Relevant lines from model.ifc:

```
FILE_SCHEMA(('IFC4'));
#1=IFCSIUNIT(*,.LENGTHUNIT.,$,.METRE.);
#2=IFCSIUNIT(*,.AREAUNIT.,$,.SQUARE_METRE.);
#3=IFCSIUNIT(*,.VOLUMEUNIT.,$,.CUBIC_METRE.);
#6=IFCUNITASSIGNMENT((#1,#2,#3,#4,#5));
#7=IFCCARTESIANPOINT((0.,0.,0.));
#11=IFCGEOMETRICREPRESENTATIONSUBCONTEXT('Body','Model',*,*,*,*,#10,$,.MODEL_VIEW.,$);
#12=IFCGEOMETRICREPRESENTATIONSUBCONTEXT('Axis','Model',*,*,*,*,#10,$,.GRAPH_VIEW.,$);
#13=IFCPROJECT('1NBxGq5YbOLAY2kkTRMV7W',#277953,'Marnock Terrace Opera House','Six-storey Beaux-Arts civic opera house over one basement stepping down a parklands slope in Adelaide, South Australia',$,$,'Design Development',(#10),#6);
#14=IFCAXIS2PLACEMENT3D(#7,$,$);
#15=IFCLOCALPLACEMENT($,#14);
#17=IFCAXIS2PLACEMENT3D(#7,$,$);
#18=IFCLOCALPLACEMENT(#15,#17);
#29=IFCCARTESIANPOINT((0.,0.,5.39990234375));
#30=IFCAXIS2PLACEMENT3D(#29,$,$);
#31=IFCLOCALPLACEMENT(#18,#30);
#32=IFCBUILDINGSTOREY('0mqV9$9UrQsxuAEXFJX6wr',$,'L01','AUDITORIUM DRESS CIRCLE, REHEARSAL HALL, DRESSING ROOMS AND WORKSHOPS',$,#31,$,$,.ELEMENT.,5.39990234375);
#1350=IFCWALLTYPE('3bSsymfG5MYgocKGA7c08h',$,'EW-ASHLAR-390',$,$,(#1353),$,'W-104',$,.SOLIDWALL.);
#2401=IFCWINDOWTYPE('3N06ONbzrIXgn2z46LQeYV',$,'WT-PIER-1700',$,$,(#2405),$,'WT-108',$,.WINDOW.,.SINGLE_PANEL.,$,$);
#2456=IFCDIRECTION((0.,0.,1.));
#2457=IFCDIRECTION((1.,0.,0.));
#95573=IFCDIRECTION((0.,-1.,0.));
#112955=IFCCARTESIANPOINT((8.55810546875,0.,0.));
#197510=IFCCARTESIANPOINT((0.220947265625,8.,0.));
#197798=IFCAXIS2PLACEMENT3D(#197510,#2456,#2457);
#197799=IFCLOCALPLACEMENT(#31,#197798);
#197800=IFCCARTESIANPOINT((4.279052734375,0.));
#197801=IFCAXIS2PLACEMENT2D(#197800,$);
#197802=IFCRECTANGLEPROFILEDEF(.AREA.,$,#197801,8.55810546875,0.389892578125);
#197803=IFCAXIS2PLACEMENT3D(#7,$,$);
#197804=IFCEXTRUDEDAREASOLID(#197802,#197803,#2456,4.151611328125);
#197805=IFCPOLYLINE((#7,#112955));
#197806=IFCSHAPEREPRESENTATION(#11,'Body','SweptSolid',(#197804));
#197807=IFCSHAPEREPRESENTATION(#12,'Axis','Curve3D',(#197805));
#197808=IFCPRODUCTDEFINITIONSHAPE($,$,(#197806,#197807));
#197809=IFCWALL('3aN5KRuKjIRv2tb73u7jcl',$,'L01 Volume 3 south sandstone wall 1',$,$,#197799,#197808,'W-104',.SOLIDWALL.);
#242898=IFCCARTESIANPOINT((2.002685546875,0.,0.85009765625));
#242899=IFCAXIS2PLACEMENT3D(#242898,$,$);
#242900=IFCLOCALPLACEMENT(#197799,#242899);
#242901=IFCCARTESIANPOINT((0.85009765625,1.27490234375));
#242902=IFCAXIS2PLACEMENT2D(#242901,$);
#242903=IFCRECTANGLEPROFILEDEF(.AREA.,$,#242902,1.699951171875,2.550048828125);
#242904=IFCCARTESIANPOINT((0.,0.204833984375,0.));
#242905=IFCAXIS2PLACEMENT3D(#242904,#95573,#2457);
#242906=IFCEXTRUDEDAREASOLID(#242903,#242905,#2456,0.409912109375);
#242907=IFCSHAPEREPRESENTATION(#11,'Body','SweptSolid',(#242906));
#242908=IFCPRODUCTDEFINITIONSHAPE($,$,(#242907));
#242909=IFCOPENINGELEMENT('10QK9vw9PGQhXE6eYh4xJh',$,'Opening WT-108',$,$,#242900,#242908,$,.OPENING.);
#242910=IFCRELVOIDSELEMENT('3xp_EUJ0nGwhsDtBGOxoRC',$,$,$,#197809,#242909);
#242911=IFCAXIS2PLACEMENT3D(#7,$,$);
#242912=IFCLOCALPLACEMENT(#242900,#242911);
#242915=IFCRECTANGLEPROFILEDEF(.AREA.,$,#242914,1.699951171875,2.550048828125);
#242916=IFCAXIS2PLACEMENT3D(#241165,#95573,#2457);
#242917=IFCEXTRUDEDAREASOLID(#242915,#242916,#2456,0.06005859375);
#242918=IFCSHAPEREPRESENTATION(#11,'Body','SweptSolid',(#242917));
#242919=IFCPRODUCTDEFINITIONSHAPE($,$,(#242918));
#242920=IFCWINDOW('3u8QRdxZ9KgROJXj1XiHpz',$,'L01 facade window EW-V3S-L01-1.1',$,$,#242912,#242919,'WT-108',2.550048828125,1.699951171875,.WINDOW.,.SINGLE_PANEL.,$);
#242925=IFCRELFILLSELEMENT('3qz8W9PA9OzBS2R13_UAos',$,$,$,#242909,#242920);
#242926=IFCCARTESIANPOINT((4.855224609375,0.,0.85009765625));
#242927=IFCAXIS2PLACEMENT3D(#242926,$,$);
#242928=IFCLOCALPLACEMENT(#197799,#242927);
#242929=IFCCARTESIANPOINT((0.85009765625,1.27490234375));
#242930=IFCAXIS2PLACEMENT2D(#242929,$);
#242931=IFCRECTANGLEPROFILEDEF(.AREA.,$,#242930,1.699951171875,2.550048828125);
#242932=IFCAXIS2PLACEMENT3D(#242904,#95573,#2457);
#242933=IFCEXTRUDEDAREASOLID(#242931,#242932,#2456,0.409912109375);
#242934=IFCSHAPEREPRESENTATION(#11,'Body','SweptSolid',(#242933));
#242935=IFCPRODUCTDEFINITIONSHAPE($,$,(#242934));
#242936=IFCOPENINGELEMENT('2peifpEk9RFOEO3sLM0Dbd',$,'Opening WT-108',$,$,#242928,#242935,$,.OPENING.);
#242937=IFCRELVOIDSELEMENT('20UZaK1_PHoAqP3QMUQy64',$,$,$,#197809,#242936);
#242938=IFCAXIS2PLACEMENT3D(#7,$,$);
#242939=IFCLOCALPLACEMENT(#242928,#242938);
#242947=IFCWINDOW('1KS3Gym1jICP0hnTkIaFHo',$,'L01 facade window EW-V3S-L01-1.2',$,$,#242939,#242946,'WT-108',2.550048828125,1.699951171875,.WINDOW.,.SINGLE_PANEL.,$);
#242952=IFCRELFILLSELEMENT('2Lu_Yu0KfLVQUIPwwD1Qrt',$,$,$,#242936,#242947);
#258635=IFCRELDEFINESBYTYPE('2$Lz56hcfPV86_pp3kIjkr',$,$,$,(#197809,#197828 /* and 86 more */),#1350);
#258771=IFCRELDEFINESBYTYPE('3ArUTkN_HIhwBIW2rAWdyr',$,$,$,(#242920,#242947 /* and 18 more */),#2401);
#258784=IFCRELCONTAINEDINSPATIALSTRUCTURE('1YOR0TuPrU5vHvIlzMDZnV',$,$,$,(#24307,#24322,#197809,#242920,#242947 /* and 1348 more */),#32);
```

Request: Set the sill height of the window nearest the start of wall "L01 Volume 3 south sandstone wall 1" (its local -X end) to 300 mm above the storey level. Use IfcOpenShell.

```python
import numpy as np
import ifcopenshell
import ifcopenshell.api.geometry
import ifcopenshell.geom
import ifcopenshell.util.element
import ifcopenshell.util.placement
import ifcopenshell.util.shape
import ifcopenshell.util.unit

model = ifcopenshell.open("model.ifc")
unit_scale = ifcopenshell.util.unit.calculate_unit_scale(model)

window = model.by_guid("3u8QRdxZ9KgROJXj1XiHpz")
opening = window.FillsVoids[0].RelatingOpeningElement
storey = ifcopenshell.util.element.get_container(window, ifc_class="IfcBuildingStorey")
level = ifcopenshell.util.placement.get_local_placement(storey.ObjectPlacement)[2, 3]

# The opening's origin need not be at the sill, so measure its lowest point.
shape = ifcopenshell.geom.create_shape(ifcopenshell.geom.settings(), opening)
bottom = ifcopenshell.util.shape.get_shape_bottom_elevation(shape, shape.geometry) / unit_scale
dz = level + 0.3 / unit_scale - bottom

shift = np.array([0.0, 0.0, dz])
# The window is placed relative to its opening, so it follows when the opening moves.
matrix = ifcopenshell.util.placement.get_local_placement(opening.ObjectPlacement)
matrix[:3, 3] += shift
ifcopenshell.api.geometry.edit_object_placement(
    model, product=opening, matrix=matrix, is_si=False, should_transform_children=True
)

print(f"moved by {dz * unit_scale:+.3f} m")

model.write("model-out.ifc")
```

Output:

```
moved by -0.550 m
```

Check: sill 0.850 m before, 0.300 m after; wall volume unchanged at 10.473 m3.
